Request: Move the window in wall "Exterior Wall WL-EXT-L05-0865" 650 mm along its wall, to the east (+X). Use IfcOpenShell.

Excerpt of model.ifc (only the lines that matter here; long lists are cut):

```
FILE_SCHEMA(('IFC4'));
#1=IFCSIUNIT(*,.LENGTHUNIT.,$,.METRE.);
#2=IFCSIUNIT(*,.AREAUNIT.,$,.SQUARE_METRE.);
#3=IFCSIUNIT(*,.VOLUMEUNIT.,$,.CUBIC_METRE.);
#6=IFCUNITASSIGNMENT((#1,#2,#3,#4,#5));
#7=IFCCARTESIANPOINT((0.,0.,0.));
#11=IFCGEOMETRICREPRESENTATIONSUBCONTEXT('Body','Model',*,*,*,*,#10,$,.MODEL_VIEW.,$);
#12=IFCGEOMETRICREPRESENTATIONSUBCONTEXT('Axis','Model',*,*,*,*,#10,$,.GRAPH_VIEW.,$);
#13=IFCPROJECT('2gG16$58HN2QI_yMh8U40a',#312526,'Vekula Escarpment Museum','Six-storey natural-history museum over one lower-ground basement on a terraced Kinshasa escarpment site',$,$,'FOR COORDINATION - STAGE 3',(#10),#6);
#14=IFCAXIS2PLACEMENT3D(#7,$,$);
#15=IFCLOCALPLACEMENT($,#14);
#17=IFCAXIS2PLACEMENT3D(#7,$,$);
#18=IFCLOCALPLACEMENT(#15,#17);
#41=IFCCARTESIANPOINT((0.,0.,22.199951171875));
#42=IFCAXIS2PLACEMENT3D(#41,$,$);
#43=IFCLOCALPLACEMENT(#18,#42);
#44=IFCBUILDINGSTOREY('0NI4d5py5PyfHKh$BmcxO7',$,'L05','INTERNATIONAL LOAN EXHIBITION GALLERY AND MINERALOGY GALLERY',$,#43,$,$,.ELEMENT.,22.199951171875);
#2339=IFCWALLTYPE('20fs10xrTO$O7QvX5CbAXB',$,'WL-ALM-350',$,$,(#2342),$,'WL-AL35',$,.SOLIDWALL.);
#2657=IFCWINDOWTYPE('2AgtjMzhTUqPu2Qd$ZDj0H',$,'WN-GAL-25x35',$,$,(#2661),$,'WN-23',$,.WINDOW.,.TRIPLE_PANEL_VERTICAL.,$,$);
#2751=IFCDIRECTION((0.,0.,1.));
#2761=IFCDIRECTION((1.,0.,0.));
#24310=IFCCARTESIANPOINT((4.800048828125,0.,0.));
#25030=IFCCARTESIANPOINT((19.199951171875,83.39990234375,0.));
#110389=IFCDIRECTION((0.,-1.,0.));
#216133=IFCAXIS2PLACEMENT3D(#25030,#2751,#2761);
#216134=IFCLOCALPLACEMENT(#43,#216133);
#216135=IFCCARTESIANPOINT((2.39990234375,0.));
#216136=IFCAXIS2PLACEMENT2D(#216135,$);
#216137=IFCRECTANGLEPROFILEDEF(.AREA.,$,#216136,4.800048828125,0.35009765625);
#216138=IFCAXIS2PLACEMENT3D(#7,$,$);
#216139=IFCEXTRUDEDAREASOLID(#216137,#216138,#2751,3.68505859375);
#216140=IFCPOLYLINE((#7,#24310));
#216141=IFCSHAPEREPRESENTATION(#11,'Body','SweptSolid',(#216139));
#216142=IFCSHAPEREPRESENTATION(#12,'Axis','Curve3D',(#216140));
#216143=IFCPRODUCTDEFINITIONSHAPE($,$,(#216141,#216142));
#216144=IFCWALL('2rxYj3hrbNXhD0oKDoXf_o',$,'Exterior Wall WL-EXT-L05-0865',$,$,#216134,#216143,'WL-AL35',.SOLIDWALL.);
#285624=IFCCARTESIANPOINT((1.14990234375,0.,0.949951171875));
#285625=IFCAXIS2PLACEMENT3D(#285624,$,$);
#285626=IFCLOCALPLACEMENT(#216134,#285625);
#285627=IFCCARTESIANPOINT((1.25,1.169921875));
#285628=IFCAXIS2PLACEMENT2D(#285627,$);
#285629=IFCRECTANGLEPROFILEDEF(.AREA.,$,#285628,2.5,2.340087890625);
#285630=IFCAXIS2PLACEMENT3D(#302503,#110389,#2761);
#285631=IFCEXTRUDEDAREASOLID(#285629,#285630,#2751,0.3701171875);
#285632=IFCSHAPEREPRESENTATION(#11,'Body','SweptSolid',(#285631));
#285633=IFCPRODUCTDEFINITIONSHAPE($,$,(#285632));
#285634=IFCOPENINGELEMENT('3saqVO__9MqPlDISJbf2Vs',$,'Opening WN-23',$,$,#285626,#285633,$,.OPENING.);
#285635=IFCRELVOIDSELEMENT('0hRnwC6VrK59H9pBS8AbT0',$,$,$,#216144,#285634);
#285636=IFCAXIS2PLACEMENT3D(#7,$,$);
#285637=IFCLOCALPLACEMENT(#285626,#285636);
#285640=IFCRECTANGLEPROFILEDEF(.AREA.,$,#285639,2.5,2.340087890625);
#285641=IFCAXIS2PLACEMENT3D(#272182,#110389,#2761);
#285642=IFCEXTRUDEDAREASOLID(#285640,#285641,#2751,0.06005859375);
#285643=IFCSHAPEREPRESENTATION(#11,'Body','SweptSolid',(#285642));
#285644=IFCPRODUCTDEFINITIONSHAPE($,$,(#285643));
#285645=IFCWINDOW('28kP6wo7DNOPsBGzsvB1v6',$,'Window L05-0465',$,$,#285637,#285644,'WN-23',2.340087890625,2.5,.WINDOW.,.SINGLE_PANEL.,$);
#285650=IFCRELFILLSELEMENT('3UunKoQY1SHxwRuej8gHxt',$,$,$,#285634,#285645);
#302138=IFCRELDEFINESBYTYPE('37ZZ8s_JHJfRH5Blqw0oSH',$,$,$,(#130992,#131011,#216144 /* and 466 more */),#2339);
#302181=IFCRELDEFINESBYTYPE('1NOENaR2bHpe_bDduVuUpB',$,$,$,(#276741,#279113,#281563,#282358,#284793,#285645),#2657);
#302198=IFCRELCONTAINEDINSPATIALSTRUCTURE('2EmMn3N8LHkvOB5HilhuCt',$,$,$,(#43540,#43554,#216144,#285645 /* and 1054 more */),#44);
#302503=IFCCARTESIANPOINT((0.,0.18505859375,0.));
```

```python
import ifcopenshell
import ifcopenshell.api.geometry
import ifcopenshell.util.placement

model = ifcopenshell.open("model.ifc")

window = model.by_guid("28kP6wo7DNOPsBGzsvB1v6")
opening = window.FillsVoids[0].RelatingOpeningElement
wall = opening.VoidsElements[0].RelatingBuildingElement

wall_matrix = ifcopenshell.util.placement.get_local_placement(wall.ObjectPlacement)
shift = wall_matrix[:3, 0] * 0.65
before = ifcopenshell.util.placement.get_local_placement(window.ObjectPlacement)[:3, 3].copy()

# The window is placed relative to its opening, so it follows when the opening moves.
matrix = ifcopenshell.util.placement.get_local_placement(opening.ObjectPlacement)
matrix[:3, 3] += shift
ifcopenshell.api.geometry.edit_object_placement(
    model, product=opening, matrix=matrix, is_si=False, should_transform_children=True
)

after = ifcopenshell.util.placement.get_local_placement(window.ObjectPlacement)[:3, 3]
print("window moved by", (after - before).round(3) + 0.0)

model.write("model-out.ifc")
```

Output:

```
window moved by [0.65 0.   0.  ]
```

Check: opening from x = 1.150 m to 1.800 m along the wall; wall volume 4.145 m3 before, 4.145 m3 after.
